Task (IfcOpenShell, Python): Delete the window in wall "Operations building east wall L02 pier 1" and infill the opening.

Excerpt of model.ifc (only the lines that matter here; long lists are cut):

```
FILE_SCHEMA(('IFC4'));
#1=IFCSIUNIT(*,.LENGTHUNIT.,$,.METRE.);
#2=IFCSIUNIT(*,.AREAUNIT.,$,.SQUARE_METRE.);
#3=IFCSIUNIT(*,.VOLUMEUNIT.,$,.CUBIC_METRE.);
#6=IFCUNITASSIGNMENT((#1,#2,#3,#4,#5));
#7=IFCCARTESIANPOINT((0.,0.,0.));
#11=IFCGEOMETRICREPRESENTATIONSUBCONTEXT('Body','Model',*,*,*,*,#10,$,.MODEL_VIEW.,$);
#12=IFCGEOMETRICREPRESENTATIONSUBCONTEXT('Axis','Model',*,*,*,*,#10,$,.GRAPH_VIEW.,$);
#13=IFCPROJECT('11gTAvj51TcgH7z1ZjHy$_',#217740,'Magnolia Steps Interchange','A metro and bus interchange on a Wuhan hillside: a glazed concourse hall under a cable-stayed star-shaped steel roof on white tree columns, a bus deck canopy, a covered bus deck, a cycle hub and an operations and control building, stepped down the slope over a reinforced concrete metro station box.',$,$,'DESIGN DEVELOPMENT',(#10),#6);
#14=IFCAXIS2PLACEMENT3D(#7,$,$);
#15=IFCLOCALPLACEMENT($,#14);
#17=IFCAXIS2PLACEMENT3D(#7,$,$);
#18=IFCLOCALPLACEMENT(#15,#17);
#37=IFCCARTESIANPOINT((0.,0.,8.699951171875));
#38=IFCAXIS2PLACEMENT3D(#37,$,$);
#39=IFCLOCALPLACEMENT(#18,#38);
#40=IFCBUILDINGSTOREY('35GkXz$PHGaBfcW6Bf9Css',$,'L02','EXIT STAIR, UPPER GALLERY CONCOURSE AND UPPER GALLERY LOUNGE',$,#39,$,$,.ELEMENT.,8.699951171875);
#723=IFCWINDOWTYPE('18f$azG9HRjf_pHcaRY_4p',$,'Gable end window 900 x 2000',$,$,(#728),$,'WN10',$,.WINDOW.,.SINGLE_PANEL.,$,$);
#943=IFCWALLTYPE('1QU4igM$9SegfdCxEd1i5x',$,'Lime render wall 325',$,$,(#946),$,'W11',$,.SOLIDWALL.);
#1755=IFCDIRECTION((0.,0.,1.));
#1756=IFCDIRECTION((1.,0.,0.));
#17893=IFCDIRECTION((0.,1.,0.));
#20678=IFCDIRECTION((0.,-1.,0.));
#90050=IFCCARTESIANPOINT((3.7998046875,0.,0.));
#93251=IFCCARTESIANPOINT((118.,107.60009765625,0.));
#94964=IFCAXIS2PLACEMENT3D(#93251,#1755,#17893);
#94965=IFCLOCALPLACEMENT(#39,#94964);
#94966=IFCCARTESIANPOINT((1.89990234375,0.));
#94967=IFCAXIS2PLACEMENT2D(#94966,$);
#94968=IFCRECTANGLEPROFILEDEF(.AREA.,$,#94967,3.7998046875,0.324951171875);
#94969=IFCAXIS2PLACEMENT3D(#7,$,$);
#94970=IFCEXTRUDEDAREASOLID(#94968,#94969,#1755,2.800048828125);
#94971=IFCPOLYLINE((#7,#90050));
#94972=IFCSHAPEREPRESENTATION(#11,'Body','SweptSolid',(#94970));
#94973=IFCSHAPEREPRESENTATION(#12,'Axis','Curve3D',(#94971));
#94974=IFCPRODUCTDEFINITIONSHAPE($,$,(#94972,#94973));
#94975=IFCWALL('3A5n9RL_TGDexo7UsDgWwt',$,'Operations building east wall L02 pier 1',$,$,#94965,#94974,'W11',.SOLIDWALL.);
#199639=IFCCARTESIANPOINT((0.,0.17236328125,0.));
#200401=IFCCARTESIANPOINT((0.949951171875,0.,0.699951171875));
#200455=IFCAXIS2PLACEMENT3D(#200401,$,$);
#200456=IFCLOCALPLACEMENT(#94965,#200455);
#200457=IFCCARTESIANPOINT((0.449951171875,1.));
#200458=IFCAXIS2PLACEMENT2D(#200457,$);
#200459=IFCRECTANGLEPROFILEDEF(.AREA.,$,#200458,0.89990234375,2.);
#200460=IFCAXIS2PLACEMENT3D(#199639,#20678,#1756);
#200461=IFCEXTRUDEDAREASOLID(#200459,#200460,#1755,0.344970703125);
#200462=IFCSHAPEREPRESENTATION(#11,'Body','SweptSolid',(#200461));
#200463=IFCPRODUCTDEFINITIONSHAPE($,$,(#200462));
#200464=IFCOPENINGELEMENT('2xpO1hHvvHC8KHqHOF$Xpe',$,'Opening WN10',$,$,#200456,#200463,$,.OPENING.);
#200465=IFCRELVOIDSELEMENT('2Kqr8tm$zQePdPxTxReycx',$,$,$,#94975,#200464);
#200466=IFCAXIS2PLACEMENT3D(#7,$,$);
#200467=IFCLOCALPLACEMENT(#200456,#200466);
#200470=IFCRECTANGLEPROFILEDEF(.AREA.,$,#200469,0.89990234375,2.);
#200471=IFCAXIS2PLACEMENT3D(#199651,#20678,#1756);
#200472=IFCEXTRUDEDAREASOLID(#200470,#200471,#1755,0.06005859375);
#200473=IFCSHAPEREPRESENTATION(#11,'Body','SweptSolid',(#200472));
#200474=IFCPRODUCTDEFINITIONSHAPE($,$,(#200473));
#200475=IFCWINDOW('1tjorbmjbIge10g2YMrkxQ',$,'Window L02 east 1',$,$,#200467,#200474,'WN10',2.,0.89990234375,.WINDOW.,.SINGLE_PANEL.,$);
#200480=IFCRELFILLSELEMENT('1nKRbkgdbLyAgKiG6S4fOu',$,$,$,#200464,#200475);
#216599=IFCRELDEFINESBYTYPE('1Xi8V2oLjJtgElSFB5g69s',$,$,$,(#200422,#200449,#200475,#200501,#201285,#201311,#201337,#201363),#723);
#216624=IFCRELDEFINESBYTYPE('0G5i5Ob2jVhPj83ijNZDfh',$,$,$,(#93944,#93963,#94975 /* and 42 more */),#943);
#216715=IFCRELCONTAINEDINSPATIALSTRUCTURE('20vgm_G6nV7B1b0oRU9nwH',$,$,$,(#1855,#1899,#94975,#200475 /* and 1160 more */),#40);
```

```python
import ifcopenshell
import ifcopenshell.api.feature
import ifcopenshell.api.root
import ifcopenshell.geom
import ifcopenshell.util.shape

model = ifcopenshell.open("model.ifc")
settings = ifcopenshell.geom.settings()


def volume(element):
    """Net volume in cubic metres, openings subtracted."""
    shape = ifcopenshell.geom.create_shape(settings, element)
    return ifcopenshell.util.shape.get_volume(shape.geometry)


window = model.by_id(200475)
opening = window.FillsVoids[0].RelatingOpeningElement
wall = opening.VoidsElements[0].RelatingBuildingElement
before = volume(wall)

ifcopenshell.api.root.remove_product(model, product=window)
ifcopenshell.api.feature.remove_feature(model, feature=opening)

after = volume(wall)

print(f"wall volume {before:.3f} -> {after:.3f} m3")

model.write("model-out.ifc")
```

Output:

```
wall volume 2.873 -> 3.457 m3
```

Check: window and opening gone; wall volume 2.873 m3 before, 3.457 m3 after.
